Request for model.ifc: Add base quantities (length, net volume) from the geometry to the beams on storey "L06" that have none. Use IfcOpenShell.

First a look at what the model holds.

```python
import ifcopenshell
import ifcopenshell.util.element
import ifcopenshell.util.unit

model = ifcopenshell.open("model.ifc")
print(model.schema)
for unit_type in ("LENGTHUNIT", "AREAUNIT", "VOLUMEUNIT"):
    print(unit_type, ifcopenshell.util.unit.calculate_unit_scale(model, unit_type))
storey = next(s for s in model.by_type("IfcBuildingStorey") if s.Name == "L06")
beams = [e for e in ifcopenshell.util.element.get_decomposition(storey) if e.is_a("IfcBeam")]
for e in sorted(beams, key=lambda e: e.id()):
    print(e.id(), e.is_a(), e.Name, list(ifcopenshell.util.element.get_psets(e, qtos_only=True)), sep=" | ")
```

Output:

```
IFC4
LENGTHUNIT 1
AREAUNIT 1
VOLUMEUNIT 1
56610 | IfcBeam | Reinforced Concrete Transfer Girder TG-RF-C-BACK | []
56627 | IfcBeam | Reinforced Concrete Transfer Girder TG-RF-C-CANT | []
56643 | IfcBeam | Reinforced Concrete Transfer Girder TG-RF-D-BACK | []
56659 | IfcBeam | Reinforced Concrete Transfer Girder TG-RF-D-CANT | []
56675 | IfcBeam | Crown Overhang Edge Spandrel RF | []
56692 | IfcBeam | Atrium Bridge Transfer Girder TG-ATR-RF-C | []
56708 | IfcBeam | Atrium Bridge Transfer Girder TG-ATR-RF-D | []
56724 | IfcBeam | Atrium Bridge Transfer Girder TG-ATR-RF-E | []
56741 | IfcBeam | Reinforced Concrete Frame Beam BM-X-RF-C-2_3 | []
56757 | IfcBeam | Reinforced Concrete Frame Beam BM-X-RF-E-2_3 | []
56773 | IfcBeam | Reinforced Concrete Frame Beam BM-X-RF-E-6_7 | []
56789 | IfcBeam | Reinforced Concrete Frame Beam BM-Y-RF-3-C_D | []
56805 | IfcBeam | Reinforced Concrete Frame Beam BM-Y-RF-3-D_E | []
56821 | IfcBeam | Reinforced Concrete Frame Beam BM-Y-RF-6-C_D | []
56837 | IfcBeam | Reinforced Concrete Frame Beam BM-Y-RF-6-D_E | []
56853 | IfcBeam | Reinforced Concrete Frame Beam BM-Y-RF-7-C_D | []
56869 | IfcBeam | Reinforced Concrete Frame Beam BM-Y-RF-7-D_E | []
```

```python
import ifcopenshell
import ifcopenshell.api.pset
import ifcopenshell.geom
import ifcopenshell.util.element
import ifcopenshell.util.shape
import ifcopenshell.util.unit

model = ifcopenshell.open("model.ifc")
unit_scale = ifcopenshell.util.unit.calculate_unit_scale(model)
volume_scale = ifcopenshell.util.unit.calculate_unit_scale(model, "VOLUMEUNIT")
settings = ifcopenshell.geom.settings()

storey = next(s for s in model.by_type("IfcBuildingStorey") if s.Name == "L06")
beams = [e for e in ifcopenshell.util.element.get_decomposition(storey) if e.is_a("IfcBeam")]

for e in sorted(beams, key=lambda e: e.id()):
    if ifcopenshell.util.element.get_psets(e, qtos_only=True, should_inherit=False):
        continue
    # Geometry comes back in metres, in the element's own axes.
    shape = ifcopenshell.geom.create_shape(settings, e)
    values = {
        "Length": ifcopenshell.util.shape.get_max_xyz(shape.geometry) / unit_scale,
        "NetVolume": ifcopenshell.util.shape.get_volume(shape.geometry) / volume_scale,
    }
    qto = ifcopenshell.api.pset.add_qto(model, product=e, name="Qto_BeamBaseQuantities")
    ifcopenshell.api.pset.edit_qto(model, qto=qto, properties=values)
    print(e.id(), {k: round(v, 3) for k, v in values.items()})

model.write("model_updated.ifc")
```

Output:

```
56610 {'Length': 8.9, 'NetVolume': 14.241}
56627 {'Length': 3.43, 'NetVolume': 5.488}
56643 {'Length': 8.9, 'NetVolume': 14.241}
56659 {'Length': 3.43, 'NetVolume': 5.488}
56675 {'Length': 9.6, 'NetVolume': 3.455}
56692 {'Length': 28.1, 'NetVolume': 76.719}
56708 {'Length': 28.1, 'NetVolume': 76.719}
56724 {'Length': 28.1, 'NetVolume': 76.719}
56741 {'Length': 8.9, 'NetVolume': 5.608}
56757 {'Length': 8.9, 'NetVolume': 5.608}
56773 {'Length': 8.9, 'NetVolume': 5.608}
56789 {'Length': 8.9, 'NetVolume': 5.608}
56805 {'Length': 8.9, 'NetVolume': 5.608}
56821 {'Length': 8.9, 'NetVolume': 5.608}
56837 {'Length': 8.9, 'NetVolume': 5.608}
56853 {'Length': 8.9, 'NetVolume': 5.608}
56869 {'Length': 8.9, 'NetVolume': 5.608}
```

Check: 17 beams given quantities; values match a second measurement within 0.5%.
